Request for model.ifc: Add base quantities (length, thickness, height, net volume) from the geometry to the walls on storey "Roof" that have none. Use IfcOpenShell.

First a look at what the model holds.

```python
import ifcopenshell
import ifcopenshell.util.element
import ifcopenshell.util.unit

model = ifcopenshell.open("model.ifc")
print(model.schema)
for unit_type in ("LENGTHUNIT", "AREAUNIT", "VOLUMEUNIT"):
    print(unit_type, ifcopenshell.util.unit.calculate_unit_scale(model, unit_type))
storey = next(s for s in model.by_type("IfcBuildingStorey") if s.Name == "Roof")
walls = [e for e in ifcopenshell.util.element.get_decomposition(storey) if e.is_a("IfcWall")]
for e in sorted(walls, key=lambda e: e.id()):
    print(e.id(), e.is_a(), e.Name, list(ifcopenshell.util.element.get_psets(e, qtos_only=True)), sep=" | ")
```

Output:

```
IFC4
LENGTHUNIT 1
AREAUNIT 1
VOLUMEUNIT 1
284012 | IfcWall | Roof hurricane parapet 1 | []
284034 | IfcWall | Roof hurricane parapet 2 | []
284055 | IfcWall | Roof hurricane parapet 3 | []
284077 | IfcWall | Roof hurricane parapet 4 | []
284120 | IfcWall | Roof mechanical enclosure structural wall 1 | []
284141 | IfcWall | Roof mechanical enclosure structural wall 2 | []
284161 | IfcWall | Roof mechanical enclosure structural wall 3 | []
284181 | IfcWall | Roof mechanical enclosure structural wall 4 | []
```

```python
import ifcopenshell
import ifcopenshell.api.pset
import ifcopenshell.geom
import ifcopenshell.util.element
import ifcopenshell.util.shape
import ifcopenshell.util.unit

model = ifcopenshell.open("model.ifc")
unit_scale = ifcopenshell.util.unit.calculate_unit_scale(model)
volume_scale = ifcopenshell.util.unit.calculate_unit_scale(model, "VOLUMEUNIT")
settings = ifcopenshell.geom.settings()

storey = next(s for s in model.by_type("IfcBuildingStorey") if s.Name == "Roof")
walls = [e for e in ifcopenshell.util.element.get_decomposition(storey) if e.is_a("IfcWall")]

for e in sorted(walls, key=lambda e: e.id()):
    if ifcopenshell.util.element.get_psets(e, qtos_only=True, should_inherit=False):
        continue
    # Geometry comes back in metres, in the element's own axes.
    shape = ifcopenshell.geom.create_shape(settings, e)
    values = {
        "Length": ifcopenshell.util.shape.get_x(shape.geometry) / unit_scale,
        "Width": ifcopenshell.util.shape.get_y(shape.geometry) / unit_scale,
        "Height": ifcopenshell.util.shape.get_z(shape.geometry) / unit_scale,
        "NetVolume": ifcopenshell.util.shape.get_volume(shape.geometry) / volume_scale,
    }
    qto = ifcopenshell.api.pset.add_qto(model, product=e, name="Qto_WallBaseQuantities")
    ifcopenshell.api.pset.edit_qto(model, qto=qto, properties=values)
    print(e.id(), {k: round(v, 3) for k, v in values.items()})

model.write("model_rev.ifc")
```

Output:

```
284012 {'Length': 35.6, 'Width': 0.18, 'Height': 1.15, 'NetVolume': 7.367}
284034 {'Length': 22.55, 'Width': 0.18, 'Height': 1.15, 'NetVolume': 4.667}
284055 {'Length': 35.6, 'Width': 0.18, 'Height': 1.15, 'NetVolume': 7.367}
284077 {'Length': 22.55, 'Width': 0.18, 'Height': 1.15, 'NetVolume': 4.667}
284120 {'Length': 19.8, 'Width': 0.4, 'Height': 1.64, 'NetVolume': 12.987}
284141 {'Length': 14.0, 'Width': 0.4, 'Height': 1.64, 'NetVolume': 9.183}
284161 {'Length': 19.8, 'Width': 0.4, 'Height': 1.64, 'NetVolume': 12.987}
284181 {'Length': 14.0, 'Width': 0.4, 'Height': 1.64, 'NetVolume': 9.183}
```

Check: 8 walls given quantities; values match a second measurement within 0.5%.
